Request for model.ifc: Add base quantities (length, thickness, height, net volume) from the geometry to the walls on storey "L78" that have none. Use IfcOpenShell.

First a look at what the model holds.

```python
import ifcopenshell
import ifcopenshell.util.element
import ifcopenshell.util.unit

model = ifcopenshell.open("model.ifc")
print(model.schema)
for unit_type in ("LENGTHUNIT", "AREAUNIT", "VOLUMEUNIT"):
    print(unit_type, ifcopenshell.util.unit.calculate_unit_scale(model, unit_type))
storey = next(s for s in model.by_type("IfcBuildingStorey") if s.Name == "L78")
walls = [e for e in ifcopenshell.util.element.get_decomposition(storey) if e.is_a("IfcWall")]
for e in sorted(walls, key=lambda e: e.id()):
    print(e.id(), e.is_a(), e.Name, list(ifcopenshell.util.element.get_psets(e, qtos_only=True)), sep=" | ")
```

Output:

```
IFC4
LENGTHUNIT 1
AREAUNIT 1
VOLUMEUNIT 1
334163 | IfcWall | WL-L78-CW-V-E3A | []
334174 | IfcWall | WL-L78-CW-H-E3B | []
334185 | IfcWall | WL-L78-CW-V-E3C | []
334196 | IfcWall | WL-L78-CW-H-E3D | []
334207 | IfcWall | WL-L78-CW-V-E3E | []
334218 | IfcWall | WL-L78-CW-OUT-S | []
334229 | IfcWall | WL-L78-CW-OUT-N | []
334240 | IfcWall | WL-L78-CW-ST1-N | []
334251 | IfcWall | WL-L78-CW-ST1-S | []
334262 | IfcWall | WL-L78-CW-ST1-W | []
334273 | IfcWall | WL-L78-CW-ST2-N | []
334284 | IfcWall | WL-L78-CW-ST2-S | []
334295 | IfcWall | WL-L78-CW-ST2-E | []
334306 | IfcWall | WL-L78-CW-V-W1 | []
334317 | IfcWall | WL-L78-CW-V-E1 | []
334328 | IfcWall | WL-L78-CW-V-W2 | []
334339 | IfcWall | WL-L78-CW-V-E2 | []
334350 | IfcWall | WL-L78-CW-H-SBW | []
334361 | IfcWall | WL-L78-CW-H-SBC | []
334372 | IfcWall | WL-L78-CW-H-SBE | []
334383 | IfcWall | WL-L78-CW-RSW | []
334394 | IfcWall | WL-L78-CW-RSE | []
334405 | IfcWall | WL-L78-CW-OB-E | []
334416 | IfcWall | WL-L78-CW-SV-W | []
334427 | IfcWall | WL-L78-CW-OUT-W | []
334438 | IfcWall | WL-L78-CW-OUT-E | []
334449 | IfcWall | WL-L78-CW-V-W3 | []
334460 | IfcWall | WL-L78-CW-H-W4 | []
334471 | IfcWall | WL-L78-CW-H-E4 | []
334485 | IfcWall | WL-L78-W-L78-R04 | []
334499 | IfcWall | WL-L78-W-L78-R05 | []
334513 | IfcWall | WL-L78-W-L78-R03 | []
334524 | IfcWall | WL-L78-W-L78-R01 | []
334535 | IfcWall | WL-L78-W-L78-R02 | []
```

```python
import ifcopenshell
import ifcopenshell.api.pset
import ifcopenshell.geom
import ifcopenshell.util.element
import ifcopenshell.util.shape
import ifcopenshell.util.unit

model = ifcopenshell.open("model.ifc")
unit_scale = ifcopenshell.util.unit.calculate_unit_scale(model)
volume_scale = ifcopenshell.util.unit.calculate_unit_scale(model, "VOLUMEUNIT")
settings = ifcopenshell.geom.settings()

storey = next(s for s in model.by_type("IfcBuildingStorey") if s.Name == "L78")
walls = [e for e in ifcopenshell.util.element.get_decomposition(storey) if e.is_a("IfcWall")]

for e in sorted(walls, key=lambda e: e.id()):
    if ifcopenshell.util.element.get_psets(e, qtos_only=True, should_inherit=False):
        continue
    # Geometry comes back in metres, in the element's own axes.
    shape = ifcopenshell.geom.create_shape(settings, e)
    values = {
        "Length": ifcopenshell.util.shape.get_x(shape.geometry) / unit_scale,
        "Width": ifcopenshell.util.shape.get_y(shape.geometry) / unit_scale,
        "Height": ifcopenshell.util.shape.get_z(shape.geometry) / unit_scale,
        "NetVolume": ifcopenshell.util.shape.get_volume(shape.geometry) / volume_scale,
    }
    qto = ifcopenshell.api.pset.add_qto(model, product=e, name="Qto_WallBaseQuantities")
    ifcopenshell.api.pset.edit_qto(model, qto=qto, properties=values)
    print(e.id(), {k: round(v, 3) for k, v in values.items()})

model.write("model_updated.ifc")
```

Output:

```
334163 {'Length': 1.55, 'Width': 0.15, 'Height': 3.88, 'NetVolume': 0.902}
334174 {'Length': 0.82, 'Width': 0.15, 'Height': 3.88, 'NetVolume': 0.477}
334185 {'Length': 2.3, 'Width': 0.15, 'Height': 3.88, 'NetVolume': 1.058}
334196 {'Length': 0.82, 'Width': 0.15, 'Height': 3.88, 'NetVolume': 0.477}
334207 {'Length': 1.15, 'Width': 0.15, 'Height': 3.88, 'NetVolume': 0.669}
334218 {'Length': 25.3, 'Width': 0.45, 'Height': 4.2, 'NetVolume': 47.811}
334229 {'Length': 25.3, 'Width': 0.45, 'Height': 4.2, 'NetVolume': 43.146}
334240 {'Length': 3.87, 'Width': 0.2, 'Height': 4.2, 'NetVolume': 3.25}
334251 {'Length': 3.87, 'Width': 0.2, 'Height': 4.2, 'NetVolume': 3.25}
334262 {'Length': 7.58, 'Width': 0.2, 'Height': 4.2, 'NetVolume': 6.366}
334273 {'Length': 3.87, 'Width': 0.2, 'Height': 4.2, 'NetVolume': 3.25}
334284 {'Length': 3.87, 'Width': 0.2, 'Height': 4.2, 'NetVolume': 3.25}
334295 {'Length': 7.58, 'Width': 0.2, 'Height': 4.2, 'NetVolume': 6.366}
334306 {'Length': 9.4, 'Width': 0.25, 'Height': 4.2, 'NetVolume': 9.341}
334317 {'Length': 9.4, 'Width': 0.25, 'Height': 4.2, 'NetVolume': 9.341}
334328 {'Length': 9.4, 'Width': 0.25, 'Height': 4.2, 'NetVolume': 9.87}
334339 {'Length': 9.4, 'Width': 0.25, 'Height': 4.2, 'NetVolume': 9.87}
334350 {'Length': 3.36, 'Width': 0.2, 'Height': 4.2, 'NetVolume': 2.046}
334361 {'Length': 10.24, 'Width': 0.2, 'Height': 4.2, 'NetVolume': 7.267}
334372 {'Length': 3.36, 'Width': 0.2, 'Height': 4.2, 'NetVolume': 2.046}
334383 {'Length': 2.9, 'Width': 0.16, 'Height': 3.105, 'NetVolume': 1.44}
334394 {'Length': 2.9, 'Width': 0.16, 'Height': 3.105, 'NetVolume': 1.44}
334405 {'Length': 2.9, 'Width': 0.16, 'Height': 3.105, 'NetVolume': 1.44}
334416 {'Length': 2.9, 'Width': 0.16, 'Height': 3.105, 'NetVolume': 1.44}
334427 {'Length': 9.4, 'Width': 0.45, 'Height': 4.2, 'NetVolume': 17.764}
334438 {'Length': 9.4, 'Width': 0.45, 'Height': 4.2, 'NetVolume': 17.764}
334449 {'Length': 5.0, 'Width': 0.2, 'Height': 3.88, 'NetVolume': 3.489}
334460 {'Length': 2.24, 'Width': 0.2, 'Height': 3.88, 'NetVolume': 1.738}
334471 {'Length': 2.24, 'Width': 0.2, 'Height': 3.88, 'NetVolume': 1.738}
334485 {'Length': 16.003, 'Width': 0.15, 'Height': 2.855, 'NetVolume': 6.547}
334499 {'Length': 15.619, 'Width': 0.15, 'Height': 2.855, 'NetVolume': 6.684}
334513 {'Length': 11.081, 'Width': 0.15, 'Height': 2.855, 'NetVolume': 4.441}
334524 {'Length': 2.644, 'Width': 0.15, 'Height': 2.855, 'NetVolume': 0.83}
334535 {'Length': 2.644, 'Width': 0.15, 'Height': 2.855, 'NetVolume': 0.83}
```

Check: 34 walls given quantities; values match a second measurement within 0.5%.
